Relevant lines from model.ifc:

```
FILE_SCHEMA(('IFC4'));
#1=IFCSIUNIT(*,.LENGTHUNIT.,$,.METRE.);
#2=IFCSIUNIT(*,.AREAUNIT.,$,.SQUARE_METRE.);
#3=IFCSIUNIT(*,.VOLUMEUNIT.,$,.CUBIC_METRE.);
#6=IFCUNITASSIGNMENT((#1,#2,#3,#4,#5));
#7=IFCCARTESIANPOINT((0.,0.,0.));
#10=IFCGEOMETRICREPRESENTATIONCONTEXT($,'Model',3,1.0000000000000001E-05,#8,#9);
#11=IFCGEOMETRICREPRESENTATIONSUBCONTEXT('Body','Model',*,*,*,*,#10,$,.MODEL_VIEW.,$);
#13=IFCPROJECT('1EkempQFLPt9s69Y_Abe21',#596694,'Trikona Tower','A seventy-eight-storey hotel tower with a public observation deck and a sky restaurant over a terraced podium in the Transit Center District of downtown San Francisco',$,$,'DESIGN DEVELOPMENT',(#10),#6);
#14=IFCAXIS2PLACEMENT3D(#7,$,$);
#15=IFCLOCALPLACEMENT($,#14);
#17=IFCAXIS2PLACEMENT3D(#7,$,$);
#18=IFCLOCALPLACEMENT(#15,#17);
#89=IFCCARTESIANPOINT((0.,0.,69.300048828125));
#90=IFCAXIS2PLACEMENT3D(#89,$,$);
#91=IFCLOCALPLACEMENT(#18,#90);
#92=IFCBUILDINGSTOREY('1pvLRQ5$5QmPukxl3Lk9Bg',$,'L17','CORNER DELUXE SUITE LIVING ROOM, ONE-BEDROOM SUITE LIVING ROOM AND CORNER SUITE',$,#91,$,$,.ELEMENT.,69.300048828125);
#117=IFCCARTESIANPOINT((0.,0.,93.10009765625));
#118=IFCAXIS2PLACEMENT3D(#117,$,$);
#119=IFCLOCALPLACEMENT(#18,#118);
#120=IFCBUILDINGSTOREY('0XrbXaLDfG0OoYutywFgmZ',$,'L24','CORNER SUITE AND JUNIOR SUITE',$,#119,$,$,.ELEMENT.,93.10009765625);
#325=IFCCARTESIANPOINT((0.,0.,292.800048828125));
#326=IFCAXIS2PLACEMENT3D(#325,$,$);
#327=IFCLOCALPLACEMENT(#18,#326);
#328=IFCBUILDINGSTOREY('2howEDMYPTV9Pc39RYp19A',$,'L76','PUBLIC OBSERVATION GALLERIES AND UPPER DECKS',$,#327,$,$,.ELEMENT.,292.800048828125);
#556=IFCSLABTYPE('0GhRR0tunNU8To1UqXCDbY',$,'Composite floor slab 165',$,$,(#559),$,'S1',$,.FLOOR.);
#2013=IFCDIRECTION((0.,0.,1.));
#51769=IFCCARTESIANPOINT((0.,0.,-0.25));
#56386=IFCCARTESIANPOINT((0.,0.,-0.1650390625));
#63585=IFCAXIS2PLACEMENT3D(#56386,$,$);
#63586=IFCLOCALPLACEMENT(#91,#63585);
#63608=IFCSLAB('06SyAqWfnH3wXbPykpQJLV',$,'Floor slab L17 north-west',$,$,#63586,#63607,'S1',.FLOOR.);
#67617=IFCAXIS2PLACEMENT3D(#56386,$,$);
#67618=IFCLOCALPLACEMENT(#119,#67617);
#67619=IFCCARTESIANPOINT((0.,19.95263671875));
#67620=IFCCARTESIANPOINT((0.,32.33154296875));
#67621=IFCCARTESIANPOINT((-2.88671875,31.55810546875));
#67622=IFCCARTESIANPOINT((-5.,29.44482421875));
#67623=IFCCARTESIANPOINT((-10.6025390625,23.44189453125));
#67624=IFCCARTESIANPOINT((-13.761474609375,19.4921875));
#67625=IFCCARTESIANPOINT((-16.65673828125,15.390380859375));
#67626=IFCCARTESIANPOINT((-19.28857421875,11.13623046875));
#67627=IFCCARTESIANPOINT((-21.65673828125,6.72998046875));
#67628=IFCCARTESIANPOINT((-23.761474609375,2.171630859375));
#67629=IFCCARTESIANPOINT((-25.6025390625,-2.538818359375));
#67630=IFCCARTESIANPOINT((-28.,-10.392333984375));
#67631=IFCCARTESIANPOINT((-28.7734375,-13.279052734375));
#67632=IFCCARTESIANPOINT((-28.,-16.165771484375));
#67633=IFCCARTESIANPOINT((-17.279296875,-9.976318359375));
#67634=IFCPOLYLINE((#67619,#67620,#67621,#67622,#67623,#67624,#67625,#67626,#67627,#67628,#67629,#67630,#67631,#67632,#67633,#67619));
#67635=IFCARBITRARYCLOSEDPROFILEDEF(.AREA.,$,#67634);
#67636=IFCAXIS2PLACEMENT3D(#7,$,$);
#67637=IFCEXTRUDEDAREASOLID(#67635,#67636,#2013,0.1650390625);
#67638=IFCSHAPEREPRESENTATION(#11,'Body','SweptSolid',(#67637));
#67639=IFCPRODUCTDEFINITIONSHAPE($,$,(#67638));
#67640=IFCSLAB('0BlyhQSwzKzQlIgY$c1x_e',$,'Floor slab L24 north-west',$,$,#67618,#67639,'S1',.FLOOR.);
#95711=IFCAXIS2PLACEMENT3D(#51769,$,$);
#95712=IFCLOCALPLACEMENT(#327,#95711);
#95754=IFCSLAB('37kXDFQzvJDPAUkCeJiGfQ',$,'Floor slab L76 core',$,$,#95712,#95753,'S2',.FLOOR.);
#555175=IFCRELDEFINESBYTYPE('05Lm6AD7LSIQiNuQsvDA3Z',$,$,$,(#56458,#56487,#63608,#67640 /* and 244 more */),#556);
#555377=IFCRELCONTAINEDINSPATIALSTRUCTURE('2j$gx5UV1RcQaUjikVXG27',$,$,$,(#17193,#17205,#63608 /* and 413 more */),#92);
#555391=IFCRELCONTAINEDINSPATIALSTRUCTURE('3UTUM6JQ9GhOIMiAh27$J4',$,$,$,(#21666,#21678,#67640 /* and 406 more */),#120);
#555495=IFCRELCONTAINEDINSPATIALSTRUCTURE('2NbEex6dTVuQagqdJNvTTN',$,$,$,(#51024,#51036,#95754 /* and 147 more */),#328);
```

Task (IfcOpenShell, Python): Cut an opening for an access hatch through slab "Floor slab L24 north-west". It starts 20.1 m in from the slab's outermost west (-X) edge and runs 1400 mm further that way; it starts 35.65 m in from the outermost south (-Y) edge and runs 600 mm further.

```python
import numpy as np
import ifcopenshell
import ifcopenshell.api.feature
import ifcopenshell.api.geometry
import ifcopenshell.api.root
import ifcopenshell.geom
import ifcopenshell.util.placement
import ifcopenshell.util.representation
import ifcopenshell.util.shape
import ifcopenshell.util.unit

model = ifcopenshell.open("model.ifc")
unit_scale = ifcopenshell.util.unit.calculate_unit_scale(model)
settings = ifcopenshell.geom.settings()


def volume(element):
    """Net volume in cubic metres, openings subtracted."""
    shape = ifcopenshell.geom.create_shape(settings, element)
    return ifcopenshell.util.shape.get_volume(shape.geometry)


slab = model.by_guid("0BlyhQSwzKzQlIgY$c1x_e")
before = volume(slab)

# Extent in the slab's own axes, in metres. The edges named are its -X and -Y sides.
slab_shape = ifcopenshell.geom.create_shape(settings, slab)
vertices = ifcopenshell.util.shape.get_vertices(slab_shape.geometry)
x_min, y_min, bottom = vertices.min(axis=0)
top = vertices[:, 2].max()

opening = ifcopenshell.api.root.create_entity(model, ifc_class="IfcOpeningElement", name="Access hatch opening", predefined_type="OPENING")
context = ifcopenshell.util.representation.get_context(model, "Model", "Body", "MODEL_VIEW")
width, depth = 1.4, 0.6
outline = [(0.0, 0.0), (width, 0.0), (width, depth), (0.0, depth), (0.0, 0.0)]
# Overshoot both faces by 50 mm so the cut is clean.
shape = ifcopenshell.api.geometry.add_slab_representation(
    model, context=context, depth=top - bottom + 0.1, polyline=outline
)
ifcopenshell.api.geometry.assign_representation(model, product=opening, representation=shape)

matrix = ifcopenshell.util.placement.get_local_placement(slab.ObjectPlacement)
matrix[:, 3] = matrix @ np.append(np.array([x_min + 20.1, y_min + 35.65, bottom - 0.05]) / unit_scale, 1.0)
ifcopenshell.api.geometry.edit_object_placement(model, product=opening, matrix=matrix, is_si=False)
ifcopenshell.api.feature.add_feature(model, feature=opening, element=slab)

after = volume(slab)

print(f"slab volume {before:.3f} -> {after:.3f} m3")

model.write("model-out.ifc")
```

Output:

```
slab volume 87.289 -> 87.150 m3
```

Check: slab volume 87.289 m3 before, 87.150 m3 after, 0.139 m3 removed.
